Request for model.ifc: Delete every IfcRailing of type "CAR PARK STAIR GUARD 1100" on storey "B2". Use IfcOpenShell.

First a look at what the model holds.

```python
import ifcopenshell
import ifcopenshell.util.element

model = ifcopenshell.open("model.ifc")
print(model.schema)
storey = next(s for s in model.by_type("IfcBuildingStorey") if s.Name == "B2")
railings = [e for e in ifcopenshell.util.element.get_decomposition(storey) if e.is_a("IfcRailing")]
seen = {}
for e in railings:
    element_type = ifcopenshell.util.element.get_type(e)
    name = element_type.Name if element_type not in (None, e) else None
    seen[name] = seen.get(name, 0) + 1
for name, count in sorted(seen.items(), key=str):
    print(count, "x", name)
```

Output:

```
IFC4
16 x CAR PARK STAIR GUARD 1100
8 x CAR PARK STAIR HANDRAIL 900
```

```python
import ifcopenshell
import ifcopenshell.api.root
import ifcopenshell.util.element

model = ifcopenshell.open("model.ifc")

storey = next(s for s in model.by_type("IfcBuildingStorey") if s.Name == "B2")
railings = [e for e in ifcopenshell.util.element.get_decomposition(storey) if e.is_a("IfcRailing")]
targets = [e for e in railings if (t := ifcopenshell.util.element.get_type(e)) not in (None, e) and t.Name == "CAR PARK STAIR GUARD 1100"]

for e in targets:
    ifcopenshell.api.root.remove_product(model, product=e)
print(len(targets), "removed")

model.write("model_rev.ifc")
```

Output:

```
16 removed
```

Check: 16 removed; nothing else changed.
